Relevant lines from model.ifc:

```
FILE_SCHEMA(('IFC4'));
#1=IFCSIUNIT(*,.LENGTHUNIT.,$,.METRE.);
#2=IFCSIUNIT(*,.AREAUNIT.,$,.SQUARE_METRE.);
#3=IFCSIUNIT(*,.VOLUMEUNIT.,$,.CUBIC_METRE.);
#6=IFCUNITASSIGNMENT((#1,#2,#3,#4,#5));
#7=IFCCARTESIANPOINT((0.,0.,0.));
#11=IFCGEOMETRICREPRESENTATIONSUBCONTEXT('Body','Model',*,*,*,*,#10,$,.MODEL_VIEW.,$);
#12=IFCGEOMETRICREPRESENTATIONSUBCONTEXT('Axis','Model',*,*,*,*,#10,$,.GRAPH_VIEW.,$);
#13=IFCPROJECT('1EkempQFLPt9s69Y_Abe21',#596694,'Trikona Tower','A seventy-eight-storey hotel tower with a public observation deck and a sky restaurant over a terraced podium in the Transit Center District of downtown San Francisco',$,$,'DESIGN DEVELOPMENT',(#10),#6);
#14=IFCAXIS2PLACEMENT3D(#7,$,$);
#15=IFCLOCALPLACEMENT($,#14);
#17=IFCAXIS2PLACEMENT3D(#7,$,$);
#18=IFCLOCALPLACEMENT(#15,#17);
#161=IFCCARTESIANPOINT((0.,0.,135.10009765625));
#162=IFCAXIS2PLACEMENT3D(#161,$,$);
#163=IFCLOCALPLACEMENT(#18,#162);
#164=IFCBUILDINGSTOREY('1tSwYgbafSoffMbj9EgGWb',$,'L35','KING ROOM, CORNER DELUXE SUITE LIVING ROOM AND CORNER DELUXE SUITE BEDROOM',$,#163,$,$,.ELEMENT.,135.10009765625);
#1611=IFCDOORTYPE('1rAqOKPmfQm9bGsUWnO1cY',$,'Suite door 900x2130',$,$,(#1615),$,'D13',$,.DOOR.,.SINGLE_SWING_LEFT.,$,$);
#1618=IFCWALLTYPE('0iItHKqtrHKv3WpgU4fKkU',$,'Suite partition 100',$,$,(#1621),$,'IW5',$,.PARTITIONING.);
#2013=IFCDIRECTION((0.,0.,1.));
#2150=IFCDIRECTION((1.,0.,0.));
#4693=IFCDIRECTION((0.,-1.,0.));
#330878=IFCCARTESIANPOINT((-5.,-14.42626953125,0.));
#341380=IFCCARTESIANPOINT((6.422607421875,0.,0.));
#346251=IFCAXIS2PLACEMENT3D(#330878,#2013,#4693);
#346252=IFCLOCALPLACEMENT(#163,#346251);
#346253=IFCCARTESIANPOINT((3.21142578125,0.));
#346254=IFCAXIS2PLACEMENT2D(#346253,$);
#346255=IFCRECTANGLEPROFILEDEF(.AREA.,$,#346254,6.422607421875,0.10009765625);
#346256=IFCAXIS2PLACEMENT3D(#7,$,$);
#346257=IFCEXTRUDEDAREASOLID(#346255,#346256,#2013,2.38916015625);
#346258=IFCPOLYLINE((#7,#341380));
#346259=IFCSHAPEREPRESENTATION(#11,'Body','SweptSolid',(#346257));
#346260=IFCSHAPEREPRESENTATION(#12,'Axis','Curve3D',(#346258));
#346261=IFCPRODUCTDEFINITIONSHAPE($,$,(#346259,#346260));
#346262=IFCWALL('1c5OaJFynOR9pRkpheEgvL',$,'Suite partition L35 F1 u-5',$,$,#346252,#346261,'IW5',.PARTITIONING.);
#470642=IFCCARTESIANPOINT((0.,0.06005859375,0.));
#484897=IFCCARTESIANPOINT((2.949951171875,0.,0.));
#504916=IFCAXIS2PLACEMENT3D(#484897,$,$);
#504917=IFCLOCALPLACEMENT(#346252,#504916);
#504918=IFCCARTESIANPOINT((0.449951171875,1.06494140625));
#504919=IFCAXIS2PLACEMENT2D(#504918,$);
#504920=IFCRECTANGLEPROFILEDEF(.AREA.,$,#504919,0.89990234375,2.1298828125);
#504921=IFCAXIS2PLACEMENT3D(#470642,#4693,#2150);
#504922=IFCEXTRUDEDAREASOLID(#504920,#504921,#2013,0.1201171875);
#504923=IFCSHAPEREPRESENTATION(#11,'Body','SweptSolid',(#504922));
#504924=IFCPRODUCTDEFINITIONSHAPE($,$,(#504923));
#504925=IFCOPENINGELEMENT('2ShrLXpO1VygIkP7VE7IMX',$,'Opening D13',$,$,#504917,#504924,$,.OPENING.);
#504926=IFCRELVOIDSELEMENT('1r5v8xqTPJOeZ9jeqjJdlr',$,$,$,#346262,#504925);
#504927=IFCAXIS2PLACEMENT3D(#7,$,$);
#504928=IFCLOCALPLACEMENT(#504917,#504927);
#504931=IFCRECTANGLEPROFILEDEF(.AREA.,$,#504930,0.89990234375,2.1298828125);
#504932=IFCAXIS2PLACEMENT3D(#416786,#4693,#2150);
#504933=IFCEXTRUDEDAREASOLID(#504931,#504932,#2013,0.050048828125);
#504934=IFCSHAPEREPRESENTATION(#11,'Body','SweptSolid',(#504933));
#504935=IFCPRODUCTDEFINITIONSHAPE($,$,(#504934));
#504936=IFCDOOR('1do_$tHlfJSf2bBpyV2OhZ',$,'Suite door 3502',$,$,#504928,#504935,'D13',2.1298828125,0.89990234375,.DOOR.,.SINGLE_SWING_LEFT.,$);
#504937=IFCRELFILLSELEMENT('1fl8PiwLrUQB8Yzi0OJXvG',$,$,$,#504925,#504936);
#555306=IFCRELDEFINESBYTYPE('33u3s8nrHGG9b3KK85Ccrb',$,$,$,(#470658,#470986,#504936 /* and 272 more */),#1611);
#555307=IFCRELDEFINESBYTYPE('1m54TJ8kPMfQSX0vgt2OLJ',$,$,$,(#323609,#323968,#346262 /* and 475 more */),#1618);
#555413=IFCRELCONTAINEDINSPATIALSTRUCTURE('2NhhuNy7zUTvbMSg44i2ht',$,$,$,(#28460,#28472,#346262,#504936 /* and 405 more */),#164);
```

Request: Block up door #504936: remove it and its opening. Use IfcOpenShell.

```python
import ifcopenshell
import ifcopenshell.api.feature
import ifcopenshell.api.root
import ifcopenshell.geom
import ifcopenshell.util.shape

model = ifcopenshell.open("model.ifc")
settings = ifcopenshell.geom.settings()


def volume(element):
    """Net volume in cubic metres, openings subtracted."""
    shape = ifcopenshell.geom.create_shape(settings, element)
    return ifcopenshell.util.shape.get_volume(shape.geometry)


door = model.by_id(504936)
opening = door.FillsVoids[0].RelatingOpeningElement
wall = opening.VoidsElements[0].RelatingBuildingElement
before = volume(wall)

ifcopenshell.api.root.remove_product(model, product=door)
ifcopenshell.api.feature.remove_feature(model, feature=opening)

after = volume(wall)

print(f"wall volume {before:.3f} -> {after:.3f} m3")

model.write("model_v2.ifc")
```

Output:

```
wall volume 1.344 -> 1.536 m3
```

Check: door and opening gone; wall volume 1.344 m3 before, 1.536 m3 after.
